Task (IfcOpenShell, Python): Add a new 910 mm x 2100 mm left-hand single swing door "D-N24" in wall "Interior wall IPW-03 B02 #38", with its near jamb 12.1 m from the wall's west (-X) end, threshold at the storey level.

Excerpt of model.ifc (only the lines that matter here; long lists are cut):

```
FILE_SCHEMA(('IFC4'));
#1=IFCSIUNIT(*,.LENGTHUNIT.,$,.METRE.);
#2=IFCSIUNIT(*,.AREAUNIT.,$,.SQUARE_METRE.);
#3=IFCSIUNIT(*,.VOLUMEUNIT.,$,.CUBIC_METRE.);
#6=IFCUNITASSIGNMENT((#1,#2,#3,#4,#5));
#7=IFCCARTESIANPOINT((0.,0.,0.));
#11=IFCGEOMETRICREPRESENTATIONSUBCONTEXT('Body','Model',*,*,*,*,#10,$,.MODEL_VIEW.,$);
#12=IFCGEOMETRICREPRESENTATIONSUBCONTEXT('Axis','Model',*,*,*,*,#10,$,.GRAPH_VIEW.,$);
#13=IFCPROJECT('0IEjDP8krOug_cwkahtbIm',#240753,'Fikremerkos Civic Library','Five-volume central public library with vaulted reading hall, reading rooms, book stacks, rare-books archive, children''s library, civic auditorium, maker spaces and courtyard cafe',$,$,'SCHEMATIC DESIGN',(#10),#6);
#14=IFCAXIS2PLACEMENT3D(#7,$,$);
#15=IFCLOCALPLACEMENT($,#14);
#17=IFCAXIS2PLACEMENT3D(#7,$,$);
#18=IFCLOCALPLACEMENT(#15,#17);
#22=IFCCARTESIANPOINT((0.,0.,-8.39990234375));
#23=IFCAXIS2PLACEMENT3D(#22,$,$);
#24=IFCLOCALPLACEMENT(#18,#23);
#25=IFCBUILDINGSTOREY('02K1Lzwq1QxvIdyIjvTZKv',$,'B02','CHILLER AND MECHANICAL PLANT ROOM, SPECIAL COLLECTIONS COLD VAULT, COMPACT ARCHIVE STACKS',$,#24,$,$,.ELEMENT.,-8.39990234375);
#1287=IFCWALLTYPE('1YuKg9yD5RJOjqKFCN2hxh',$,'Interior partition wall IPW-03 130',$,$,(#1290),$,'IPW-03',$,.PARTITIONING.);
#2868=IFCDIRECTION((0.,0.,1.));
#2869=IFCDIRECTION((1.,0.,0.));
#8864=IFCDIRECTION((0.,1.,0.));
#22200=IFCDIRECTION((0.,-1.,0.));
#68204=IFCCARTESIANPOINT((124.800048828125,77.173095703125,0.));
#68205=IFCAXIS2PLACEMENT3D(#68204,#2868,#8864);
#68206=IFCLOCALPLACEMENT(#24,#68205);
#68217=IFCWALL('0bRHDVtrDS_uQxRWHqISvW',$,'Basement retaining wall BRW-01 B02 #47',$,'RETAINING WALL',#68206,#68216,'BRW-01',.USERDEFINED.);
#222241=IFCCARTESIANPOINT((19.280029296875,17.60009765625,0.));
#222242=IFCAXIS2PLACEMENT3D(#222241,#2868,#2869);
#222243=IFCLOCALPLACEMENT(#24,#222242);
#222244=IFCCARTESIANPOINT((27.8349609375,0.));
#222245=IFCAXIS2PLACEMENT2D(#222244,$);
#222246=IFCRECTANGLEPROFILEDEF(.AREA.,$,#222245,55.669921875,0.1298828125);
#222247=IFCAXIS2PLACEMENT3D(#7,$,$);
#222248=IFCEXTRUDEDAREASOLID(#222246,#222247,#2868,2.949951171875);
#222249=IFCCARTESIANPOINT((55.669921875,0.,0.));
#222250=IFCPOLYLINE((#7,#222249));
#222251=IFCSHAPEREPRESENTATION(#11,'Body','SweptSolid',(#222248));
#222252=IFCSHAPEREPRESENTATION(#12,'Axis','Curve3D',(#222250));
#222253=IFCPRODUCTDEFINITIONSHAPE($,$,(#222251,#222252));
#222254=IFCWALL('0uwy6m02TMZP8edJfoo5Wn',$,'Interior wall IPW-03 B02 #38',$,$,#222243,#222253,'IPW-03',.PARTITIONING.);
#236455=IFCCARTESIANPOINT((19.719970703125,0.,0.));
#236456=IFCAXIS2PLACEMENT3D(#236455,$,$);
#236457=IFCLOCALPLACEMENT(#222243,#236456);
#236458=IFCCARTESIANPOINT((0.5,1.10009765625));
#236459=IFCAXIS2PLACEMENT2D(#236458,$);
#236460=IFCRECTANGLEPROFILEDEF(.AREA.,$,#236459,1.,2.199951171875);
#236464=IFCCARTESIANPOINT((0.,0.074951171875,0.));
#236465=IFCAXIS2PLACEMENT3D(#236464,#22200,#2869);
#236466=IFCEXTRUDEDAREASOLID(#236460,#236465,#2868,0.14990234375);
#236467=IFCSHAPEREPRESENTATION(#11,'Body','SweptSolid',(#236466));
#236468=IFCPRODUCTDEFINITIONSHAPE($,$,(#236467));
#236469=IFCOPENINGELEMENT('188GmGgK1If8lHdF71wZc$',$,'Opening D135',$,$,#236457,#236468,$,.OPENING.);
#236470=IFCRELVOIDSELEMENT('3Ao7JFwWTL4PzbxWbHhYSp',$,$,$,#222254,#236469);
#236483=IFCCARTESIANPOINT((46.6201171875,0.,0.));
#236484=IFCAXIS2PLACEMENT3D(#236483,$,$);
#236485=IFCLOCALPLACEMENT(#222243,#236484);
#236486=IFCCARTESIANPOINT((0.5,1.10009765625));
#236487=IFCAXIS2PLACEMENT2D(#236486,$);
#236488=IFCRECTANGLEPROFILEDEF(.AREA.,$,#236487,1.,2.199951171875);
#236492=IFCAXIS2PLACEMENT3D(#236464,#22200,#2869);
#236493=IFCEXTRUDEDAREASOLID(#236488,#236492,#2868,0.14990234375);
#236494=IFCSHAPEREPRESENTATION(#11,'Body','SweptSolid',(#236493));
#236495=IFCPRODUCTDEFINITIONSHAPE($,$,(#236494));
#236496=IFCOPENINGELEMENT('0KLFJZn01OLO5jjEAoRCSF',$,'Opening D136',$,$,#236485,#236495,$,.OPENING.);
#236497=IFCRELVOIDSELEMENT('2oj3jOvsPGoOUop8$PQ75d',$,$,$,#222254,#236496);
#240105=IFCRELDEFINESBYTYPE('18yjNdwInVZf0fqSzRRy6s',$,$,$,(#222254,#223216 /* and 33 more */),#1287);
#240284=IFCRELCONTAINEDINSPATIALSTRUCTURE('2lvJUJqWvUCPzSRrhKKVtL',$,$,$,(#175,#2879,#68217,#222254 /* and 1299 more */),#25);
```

```python
import numpy as np
import ifcopenshell
import ifcopenshell.api.feature
import ifcopenshell.api.geometry
import ifcopenshell.api.root
import ifcopenshell.api.spatial
import ifcopenshell.geom
import ifcopenshell.util.element
import ifcopenshell.util.placement
import ifcopenshell.util.representation
import ifcopenshell.util.shape
import ifcopenshell.util.unit

model = ifcopenshell.open("model.ifc")
unit_scale = ifcopenshell.util.unit.calculate_unit_scale(model)
settings = ifcopenshell.geom.settings()


def volume(element):
    """Net volume in cubic metres, openings subtracted."""
    shape = ifcopenshell.geom.create_shape(settings, element)
    return ifcopenshell.util.shape.get_volume(shape.geometry)


wall = model.by_guid("0uwy6m02TMZP8edJfoo5Wn")
storey = ifcopenshell.util.element.get_container(wall, ifc_class="IfcBuildingStorey")
context = ifcopenshell.util.representation.get_context(model, "Model", "Body", "MODEL_VIEW")
before = volume(wall)

width, height, from_end, sill = 0.91, 2.1, 12.1, 0.0  # metres

# The wall runs along its own X axis, and the end named is its -X end.
wall_shape = ifcopenshell.geom.create_shape(settings, wall)
x, y, z = ifcopenshell.util.shape.get_vertices(wall_shape.geometry).T
start = x.min() + from_end
face, thickness = float(y.min()), float(y.max() - y.min())
wall_matrix = ifcopenshell.util.placement.get_local_placement(wall.ObjectPlacement)
level = ifcopenshell.util.placement.get_local_placement(storey.ObjectPlacement)[2, 3]


def in_wall(x, y):
    """Placement at x, y metres in the wall's axes, at sill height."""
    matrix = wall_matrix.copy()
    matrix[:, 3] = wall_matrix @ np.array([x / unit_scale, y / unit_scale, 0.0, 1.0])
    matrix[2, 3] = level + sill / unit_scale
    return matrix


# Opening: a box that overshoots both wall faces by 50 mm.
opening = ifcopenshell.api.root.create_entity(model, ifc_class="IfcOpeningElement", predefined_type="OPENING")
box = ifcopenshell.api.geometry.add_wall_representation(
    model, context=context, length=width, height=height, thickness=thickness + 0.1
)
ifcopenshell.api.geometry.assign_representation(model, product=opening, representation=box)
ifcopenshell.api.geometry.edit_object_placement(model, product=opening, matrix=in_wall(start, face - 0.05), is_si=False)
ifcopenshell.api.feature.add_feature(model, feature=opening, element=wall)

door = ifcopenshell.api.root.create_entity(model, ifc_class="IfcDoor", name="D-N24", predefined_type="DOOR")
door.OverallWidth, door.OverallHeight = width / unit_scale, height / unit_scale
door.OperationType = "SINGLE_SWING_LEFT"
body = ifcopenshell.api.geometry.add_door_representation(
    model,
    context=context,
    overall_width=door.OverallWidth,
    overall_height=door.OverallHeight,
    operation_type="SINGLE_SWING_LEFT",
    lining_properties={"LiningDepth": thickness / unit_scale, "ThresholdDepth": thickness / unit_scale},
)
ifcopenshell.api.geometry.assign_representation(model, product=door, representation=body)
ifcopenshell.api.spatial.assign_container(model, products=[door], relating_structure=storey)
ifcopenshell.api.feature.add_filling(model, opening=opening, element=door)

# The lining spans the wall, so the door starts at the wall face.
ifcopenshell.api.geometry.edit_object_placement(model, product=door, matrix=in_wall(start, face), is_si=False)

after = volume(wall)

print(f"wall volume {before:.3f} -> {after:.3f} m3")

model.write("model-out.ifc")
```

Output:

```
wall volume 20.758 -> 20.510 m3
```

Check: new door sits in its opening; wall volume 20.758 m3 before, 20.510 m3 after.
